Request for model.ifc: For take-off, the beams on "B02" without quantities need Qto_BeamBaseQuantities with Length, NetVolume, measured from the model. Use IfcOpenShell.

First a look at what the model holds.

```python
import ifcopenshell
import ifcopenshell.util.element
import ifcopenshell.util.unit

model = ifcopenshell.open("model.ifc")
print(model.schema)
for unit_type in ("LENGTHUNIT", "AREAUNIT", "VOLUMEUNIT"):
    print(unit_type, ifcopenshell.util.unit.calculate_unit_scale(model, unit_type))
storey = next(s for s in model.by_type("IfcBuildingStorey") if s.Name == "B02")
beams = [e for e in ifcopenshell.util.element.get_decomposition(storey) if e.is_a("IfcBeam")]
for e in sorted(beams, key=lambda e: e.id()):
    print(e.id(), e.is_a(), e.Name, list(ifcopenshell.util.element.get_psets(e, qtos_only=True)), sep=" | ")
```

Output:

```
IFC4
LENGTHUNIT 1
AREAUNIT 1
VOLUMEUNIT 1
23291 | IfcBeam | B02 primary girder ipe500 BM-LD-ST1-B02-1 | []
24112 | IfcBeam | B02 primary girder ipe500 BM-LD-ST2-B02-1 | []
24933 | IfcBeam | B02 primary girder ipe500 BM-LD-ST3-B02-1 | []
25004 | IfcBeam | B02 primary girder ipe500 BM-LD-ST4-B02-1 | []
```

```python
import ifcopenshell
import ifcopenshell.api.pset
import ifcopenshell.geom
import ifcopenshell.util.element
import ifcopenshell.util.shape
import ifcopenshell.util.unit

model = ifcopenshell.open("model.ifc")
unit_scale = ifcopenshell.util.unit.calculate_unit_scale(model)
volume_scale = ifcopenshell.util.unit.calculate_unit_scale(model, "VOLUMEUNIT")
settings = ifcopenshell.geom.settings()

storey = next(s for s in model.by_type("IfcBuildingStorey") if s.Name == "B02")
beams = [e for e in ifcopenshell.util.element.get_decomposition(storey) if e.is_a("IfcBeam")]

for e in sorted(beams, key=lambda e: e.id()):
    if ifcopenshell.util.element.get_psets(e, qtos_only=True, should_inherit=False):
        continue
    # Geometry comes back in metres, in the element's own axes.
    shape = ifcopenshell.geom.create_shape(settings, e)
    values = {
        "Length": ifcopenshell.util.shape.get_max_xyz(shape.geometry) / unit_scale,
        "NetVolume": ifcopenshell.util.shape.get_volume(shape.geometry) / volume_scale,
    }
    qto = ifcopenshell.api.pset.add_qto(model, product=e, name="Qto_BeamBaseQuantities")
    ifcopenshell.api.pset.edit_qto(model, qto=qto, properties=values)
    print(e.id(), {k: round(v, 3) for k, v in values.items()})

model.write("model-out.ifc")
```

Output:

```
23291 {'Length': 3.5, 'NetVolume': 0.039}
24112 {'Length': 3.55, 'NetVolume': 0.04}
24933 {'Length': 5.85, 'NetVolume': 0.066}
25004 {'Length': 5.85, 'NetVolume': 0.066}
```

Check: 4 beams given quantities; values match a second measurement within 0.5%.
